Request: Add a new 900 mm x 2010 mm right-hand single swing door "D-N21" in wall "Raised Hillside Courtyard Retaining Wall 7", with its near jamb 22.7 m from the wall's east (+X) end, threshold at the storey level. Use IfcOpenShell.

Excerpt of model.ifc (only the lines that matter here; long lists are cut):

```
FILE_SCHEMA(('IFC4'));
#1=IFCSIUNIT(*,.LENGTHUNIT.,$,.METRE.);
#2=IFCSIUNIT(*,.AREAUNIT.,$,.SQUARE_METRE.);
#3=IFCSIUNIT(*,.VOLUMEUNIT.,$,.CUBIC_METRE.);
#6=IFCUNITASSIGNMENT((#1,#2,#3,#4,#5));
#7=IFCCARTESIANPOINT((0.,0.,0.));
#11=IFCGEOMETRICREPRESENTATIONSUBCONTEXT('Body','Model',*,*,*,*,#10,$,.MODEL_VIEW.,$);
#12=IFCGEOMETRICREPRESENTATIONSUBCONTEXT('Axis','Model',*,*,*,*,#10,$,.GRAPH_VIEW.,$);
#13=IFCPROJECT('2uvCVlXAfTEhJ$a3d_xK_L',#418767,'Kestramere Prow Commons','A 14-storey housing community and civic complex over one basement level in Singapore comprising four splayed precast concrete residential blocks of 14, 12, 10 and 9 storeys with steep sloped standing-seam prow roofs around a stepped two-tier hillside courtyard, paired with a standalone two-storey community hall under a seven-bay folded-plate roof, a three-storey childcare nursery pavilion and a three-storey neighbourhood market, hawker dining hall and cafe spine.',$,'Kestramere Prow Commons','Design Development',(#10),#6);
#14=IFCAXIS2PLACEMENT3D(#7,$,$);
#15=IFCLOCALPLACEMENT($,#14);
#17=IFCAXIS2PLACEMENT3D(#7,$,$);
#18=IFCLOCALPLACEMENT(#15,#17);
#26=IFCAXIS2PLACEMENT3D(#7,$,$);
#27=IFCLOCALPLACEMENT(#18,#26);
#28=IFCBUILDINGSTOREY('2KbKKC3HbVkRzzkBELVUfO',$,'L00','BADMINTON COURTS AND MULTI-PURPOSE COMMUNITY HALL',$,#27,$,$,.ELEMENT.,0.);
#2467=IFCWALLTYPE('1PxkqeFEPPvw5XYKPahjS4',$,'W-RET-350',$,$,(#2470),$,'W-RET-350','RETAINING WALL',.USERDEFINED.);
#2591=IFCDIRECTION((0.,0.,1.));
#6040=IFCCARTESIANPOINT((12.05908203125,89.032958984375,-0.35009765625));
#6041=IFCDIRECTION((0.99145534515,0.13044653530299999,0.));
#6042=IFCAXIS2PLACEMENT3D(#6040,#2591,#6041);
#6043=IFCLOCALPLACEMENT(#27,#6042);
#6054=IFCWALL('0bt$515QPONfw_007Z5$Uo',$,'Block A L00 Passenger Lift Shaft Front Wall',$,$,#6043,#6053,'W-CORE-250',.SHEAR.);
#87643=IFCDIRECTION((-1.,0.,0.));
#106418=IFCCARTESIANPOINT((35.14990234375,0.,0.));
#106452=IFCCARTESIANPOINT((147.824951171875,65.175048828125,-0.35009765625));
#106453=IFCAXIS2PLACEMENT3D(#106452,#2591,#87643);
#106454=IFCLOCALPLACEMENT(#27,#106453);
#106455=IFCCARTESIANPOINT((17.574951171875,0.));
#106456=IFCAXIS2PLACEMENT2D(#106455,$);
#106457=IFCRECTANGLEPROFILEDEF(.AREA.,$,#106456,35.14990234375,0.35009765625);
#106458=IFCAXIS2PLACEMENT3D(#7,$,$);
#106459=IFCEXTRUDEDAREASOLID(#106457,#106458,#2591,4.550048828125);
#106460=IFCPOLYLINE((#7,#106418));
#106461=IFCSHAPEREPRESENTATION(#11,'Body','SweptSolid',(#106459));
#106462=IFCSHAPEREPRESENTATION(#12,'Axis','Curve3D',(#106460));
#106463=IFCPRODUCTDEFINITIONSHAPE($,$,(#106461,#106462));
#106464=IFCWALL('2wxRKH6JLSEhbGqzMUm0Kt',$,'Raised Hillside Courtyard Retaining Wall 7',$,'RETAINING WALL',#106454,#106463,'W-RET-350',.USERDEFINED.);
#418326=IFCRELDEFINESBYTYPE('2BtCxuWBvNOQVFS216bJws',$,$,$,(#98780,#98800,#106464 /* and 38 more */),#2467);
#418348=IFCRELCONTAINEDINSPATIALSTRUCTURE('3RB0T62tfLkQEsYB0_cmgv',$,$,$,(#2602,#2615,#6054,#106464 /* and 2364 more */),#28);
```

```python
import numpy as np
import ifcopenshell
import ifcopenshell.api.feature
import ifcopenshell.api.geometry
import ifcopenshell.api.root
import ifcopenshell.api.spatial
import ifcopenshell.geom
import ifcopenshell.util.element
import ifcopenshell.util.placement
import ifcopenshell.util.representation
import ifcopenshell.util.shape
import ifcopenshell.util.unit

model = ifcopenshell.open("model.ifc")
unit_scale = ifcopenshell.util.unit.calculate_unit_scale(model)
settings = ifcopenshell.geom.settings()


def volume(element):
    """Net volume in cubic metres, openings subtracted."""
    shape = ifcopenshell.geom.create_shape(settings, element)
    return ifcopenshell.util.shape.get_volume(shape.geometry)


wall = model.by_guid("2wxRKH6JLSEhbGqzMUm0Kt")
storey = ifcopenshell.util.element.get_container(wall, ifc_class="IfcBuildingStorey")
context = ifcopenshell.util.representation.get_context(model, "Model", "Body", "MODEL_VIEW")
before = volume(wall)

width, height, from_end, sill = 0.9, 2.01, 22.7, 0.0  # metres

# The wall runs along its own X axis, and the end named is its -X end.
wall_shape = ifcopenshell.geom.create_shape(settings, wall)
x, y, z = ifcopenshell.util.shape.get_vertices(wall_shape.geometry).T
start = x.min() + from_end
face, thickness = float(y.min()), float(y.max() - y.min())
wall_matrix = ifcopenshell.util.placement.get_local_placement(wall.ObjectPlacement)
level = ifcopenshell.util.placement.get_local_placement(storey.ObjectPlacement)[2, 3]


def in_wall(x, y):
    """Placement at x, y metres in the wall's axes, at sill height."""
    matrix = wall_matrix.copy()
    matrix[:, 3] = wall_matrix @ np.array([x / unit_scale, y / unit_scale, 0.0, 1.0])
    matrix[2, 3] = level + sill / unit_scale
    return matrix


# Opening: a box that overshoots both wall faces by 50 mm.
opening = ifcopenshell.api.root.create_entity(model, ifc_class="IfcOpeningElement", predefined_type="OPENING")
box = ifcopenshell.api.geometry.add_wall_representation(
    model, context=context, length=width, height=height, thickness=thickness + 0.1
)
ifcopenshell.api.geometry.assign_representation(model, product=opening, representation=box)
ifcopenshell.api.geometry.edit_object_placement(model, product=opening, matrix=in_wall(start, face - 0.05), is_si=False)
ifcopenshell.api.feature.add_feature(model, feature=opening, element=wall)

door = ifcopenshell.api.root.create_entity(model, ifc_class="IfcDoor", name="D-N21", predefined_type="DOOR")
door.OverallWidth, door.OverallHeight = width / unit_scale, height / unit_scale
door.OperationType = "SINGLE_SWING_RIGHT"
body = ifcopenshell.api.geometry.add_door_representation(
    model,
    context=context,
    overall_width=door.OverallWidth,
    overall_height=door.OverallHeight,
    operation_type="SINGLE_SWING_RIGHT",
    lining_properties={"LiningDepth": thickness / unit_scale, "ThresholdDepth": thickness / unit_scale},
)
ifcopenshell.api.geometry.assign_representation(model, product=door, representation=body)
ifcopenshell.api.spatial.assign_container(model, products=[door], relating_structure=storey)
ifcopenshell.api.feature.add_filling(model, opening=opening, element=door)

# The lining spans the wall, so the door starts at the wall face.
ifcopenshell.api.geometry.edit_object_placement(model, product=door, matrix=in_wall(start, face), is_si=False)

after = volume(wall)

print(f"wall volume {before:.3f} -> {after:.3f} m3")

model.write("model-out.ifc")
```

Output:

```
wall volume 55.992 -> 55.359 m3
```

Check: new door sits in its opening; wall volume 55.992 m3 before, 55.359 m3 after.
